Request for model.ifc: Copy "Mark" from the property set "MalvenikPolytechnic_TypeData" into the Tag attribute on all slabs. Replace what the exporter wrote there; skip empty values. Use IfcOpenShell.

First a look at what the model holds.

```python
import ifcopenshell
import ifcopenshell.util.element

model = ifcopenshell.open("model.ifc")
print(model.schema)
slabs = model.by_type("IfcSlab")
print(len(slabs), "slabs")
for e in slabs[:8]:
    source = ifcopenshell.util.element.get_pset(e, "MalvenikPolytechnic_TypeData", "Mark")
    target = e.Tag
    print(e.id(), repr(source), repr(target), sep=" | ")
```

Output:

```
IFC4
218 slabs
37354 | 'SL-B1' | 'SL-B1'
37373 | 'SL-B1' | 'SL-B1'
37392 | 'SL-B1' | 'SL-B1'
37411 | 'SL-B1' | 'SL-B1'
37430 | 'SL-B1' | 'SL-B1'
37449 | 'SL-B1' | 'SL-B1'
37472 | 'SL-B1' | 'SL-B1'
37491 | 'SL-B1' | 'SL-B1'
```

```python
import ifcopenshell
import ifcopenshell.util.element

model = ifcopenshell.open("model.ifc")

count = 0
for e in model.by_type("IfcSlab"):
    value = ifcopenshell.util.element.get_pset(e, "MalvenikPolytechnic_TypeData", "Mark")
    current = e.Tag
    if not value or not value.strip() or current == value:
        continue
    e.Tag = value
    count += 1

print(count, "slabs updated")

model.write("model-out.ifc")
```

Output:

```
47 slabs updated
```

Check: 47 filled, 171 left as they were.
